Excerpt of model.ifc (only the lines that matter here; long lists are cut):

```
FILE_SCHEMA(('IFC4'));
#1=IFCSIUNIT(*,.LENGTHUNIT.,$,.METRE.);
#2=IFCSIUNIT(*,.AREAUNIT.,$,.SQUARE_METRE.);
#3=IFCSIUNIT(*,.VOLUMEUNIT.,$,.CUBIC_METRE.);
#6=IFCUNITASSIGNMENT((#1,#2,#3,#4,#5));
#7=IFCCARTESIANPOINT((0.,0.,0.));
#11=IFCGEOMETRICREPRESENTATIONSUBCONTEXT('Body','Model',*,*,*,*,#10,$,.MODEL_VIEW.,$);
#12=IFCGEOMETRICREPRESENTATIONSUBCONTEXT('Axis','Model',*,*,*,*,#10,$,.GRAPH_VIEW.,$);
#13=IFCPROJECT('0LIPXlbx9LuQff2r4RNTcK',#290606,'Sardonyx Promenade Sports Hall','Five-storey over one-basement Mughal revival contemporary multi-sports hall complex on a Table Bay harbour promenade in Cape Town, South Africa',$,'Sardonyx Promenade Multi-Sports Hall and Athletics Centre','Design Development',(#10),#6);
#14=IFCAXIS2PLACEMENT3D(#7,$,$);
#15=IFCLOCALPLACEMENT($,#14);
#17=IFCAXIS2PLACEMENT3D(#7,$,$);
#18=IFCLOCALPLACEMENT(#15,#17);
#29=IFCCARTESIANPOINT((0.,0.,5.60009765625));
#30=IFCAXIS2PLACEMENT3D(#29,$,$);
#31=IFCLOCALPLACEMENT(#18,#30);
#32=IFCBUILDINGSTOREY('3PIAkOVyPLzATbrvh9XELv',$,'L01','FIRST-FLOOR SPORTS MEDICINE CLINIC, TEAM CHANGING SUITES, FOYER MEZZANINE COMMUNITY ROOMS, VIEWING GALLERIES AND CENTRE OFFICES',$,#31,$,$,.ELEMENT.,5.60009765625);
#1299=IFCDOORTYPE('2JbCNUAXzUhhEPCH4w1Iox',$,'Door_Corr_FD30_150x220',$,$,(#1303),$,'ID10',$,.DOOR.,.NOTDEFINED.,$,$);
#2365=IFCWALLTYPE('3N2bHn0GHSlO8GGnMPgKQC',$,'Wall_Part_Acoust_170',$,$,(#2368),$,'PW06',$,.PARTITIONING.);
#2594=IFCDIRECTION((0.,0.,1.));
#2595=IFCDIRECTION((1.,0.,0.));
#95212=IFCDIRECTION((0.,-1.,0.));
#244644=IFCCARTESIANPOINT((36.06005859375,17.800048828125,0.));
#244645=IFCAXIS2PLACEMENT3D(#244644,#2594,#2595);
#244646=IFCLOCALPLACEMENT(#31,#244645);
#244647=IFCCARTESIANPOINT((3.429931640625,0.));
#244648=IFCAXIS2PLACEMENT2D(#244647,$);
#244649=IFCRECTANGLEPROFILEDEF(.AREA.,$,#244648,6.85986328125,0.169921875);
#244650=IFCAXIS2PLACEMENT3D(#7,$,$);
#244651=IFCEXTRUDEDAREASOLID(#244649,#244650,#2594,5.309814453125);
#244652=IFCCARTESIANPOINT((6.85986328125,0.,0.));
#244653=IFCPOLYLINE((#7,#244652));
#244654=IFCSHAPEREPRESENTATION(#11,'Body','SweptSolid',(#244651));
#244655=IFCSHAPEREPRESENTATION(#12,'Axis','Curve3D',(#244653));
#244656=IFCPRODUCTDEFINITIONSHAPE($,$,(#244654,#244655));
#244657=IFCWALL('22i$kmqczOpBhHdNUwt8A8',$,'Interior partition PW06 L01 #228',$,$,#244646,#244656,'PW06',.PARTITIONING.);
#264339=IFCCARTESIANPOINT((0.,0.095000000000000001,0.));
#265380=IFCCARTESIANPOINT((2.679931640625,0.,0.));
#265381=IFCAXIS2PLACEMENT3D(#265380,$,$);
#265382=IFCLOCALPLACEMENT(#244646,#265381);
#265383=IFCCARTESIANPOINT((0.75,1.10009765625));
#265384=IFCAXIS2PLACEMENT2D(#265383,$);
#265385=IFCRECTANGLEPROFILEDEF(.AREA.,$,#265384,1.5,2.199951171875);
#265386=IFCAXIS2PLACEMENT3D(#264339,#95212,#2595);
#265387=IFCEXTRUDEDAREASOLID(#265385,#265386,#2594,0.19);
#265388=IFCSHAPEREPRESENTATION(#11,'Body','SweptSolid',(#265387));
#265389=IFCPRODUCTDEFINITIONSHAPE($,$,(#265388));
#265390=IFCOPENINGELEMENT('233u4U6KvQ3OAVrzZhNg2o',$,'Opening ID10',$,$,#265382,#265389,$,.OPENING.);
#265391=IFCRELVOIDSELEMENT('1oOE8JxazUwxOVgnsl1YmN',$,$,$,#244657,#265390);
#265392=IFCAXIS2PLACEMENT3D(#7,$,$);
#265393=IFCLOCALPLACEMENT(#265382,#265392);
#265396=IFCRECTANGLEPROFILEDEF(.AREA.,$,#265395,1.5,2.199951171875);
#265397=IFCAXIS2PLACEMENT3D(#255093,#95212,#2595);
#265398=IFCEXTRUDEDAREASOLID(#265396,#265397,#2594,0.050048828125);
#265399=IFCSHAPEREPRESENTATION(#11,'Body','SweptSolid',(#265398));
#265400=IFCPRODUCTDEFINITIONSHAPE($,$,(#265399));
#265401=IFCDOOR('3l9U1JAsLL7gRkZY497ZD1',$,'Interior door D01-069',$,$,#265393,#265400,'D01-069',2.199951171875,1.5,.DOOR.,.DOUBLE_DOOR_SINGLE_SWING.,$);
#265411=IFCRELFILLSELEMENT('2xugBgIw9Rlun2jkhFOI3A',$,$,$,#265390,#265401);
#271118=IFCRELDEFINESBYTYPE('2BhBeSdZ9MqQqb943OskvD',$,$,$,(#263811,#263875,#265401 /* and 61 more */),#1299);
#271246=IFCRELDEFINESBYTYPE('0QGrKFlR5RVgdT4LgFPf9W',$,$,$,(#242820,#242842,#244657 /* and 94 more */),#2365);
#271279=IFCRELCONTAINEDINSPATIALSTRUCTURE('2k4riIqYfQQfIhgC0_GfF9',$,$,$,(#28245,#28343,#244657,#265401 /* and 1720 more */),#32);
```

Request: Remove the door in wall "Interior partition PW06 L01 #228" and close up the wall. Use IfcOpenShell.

```python
import ifcopenshell
import ifcopenshell.api.feature
import ifcopenshell.api.root
import ifcopenshell.geom
import ifcopenshell.util.shape

model = ifcopenshell.open("model.ifc")
settings = ifcopenshell.geom.settings()


def volume(element):
    """Net volume in cubic metres, openings subtracted."""
    shape = ifcopenshell.geom.create_shape(settings, element)
    return ifcopenshell.util.shape.get_volume(shape.geometry)


door = model.by_guid("3l9U1JAsLL7gRkZY497ZD1")
opening = door.FillsVoids[0].RelatingOpeningElement
wall = opening.VoidsElements[0].RelatingBuildingElement
before = volume(wall)

ifcopenshell.api.root.remove_product(model, product=door)
ifcopenshell.api.feature.remove_feature(model, feature=opening)

after = volume(wall)

print(f"wall volume {before:.3f} -> {after:.3f} m3")

model.write("model_v2.ifc")
```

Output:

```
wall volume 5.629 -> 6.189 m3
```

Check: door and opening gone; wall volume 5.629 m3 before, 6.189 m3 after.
